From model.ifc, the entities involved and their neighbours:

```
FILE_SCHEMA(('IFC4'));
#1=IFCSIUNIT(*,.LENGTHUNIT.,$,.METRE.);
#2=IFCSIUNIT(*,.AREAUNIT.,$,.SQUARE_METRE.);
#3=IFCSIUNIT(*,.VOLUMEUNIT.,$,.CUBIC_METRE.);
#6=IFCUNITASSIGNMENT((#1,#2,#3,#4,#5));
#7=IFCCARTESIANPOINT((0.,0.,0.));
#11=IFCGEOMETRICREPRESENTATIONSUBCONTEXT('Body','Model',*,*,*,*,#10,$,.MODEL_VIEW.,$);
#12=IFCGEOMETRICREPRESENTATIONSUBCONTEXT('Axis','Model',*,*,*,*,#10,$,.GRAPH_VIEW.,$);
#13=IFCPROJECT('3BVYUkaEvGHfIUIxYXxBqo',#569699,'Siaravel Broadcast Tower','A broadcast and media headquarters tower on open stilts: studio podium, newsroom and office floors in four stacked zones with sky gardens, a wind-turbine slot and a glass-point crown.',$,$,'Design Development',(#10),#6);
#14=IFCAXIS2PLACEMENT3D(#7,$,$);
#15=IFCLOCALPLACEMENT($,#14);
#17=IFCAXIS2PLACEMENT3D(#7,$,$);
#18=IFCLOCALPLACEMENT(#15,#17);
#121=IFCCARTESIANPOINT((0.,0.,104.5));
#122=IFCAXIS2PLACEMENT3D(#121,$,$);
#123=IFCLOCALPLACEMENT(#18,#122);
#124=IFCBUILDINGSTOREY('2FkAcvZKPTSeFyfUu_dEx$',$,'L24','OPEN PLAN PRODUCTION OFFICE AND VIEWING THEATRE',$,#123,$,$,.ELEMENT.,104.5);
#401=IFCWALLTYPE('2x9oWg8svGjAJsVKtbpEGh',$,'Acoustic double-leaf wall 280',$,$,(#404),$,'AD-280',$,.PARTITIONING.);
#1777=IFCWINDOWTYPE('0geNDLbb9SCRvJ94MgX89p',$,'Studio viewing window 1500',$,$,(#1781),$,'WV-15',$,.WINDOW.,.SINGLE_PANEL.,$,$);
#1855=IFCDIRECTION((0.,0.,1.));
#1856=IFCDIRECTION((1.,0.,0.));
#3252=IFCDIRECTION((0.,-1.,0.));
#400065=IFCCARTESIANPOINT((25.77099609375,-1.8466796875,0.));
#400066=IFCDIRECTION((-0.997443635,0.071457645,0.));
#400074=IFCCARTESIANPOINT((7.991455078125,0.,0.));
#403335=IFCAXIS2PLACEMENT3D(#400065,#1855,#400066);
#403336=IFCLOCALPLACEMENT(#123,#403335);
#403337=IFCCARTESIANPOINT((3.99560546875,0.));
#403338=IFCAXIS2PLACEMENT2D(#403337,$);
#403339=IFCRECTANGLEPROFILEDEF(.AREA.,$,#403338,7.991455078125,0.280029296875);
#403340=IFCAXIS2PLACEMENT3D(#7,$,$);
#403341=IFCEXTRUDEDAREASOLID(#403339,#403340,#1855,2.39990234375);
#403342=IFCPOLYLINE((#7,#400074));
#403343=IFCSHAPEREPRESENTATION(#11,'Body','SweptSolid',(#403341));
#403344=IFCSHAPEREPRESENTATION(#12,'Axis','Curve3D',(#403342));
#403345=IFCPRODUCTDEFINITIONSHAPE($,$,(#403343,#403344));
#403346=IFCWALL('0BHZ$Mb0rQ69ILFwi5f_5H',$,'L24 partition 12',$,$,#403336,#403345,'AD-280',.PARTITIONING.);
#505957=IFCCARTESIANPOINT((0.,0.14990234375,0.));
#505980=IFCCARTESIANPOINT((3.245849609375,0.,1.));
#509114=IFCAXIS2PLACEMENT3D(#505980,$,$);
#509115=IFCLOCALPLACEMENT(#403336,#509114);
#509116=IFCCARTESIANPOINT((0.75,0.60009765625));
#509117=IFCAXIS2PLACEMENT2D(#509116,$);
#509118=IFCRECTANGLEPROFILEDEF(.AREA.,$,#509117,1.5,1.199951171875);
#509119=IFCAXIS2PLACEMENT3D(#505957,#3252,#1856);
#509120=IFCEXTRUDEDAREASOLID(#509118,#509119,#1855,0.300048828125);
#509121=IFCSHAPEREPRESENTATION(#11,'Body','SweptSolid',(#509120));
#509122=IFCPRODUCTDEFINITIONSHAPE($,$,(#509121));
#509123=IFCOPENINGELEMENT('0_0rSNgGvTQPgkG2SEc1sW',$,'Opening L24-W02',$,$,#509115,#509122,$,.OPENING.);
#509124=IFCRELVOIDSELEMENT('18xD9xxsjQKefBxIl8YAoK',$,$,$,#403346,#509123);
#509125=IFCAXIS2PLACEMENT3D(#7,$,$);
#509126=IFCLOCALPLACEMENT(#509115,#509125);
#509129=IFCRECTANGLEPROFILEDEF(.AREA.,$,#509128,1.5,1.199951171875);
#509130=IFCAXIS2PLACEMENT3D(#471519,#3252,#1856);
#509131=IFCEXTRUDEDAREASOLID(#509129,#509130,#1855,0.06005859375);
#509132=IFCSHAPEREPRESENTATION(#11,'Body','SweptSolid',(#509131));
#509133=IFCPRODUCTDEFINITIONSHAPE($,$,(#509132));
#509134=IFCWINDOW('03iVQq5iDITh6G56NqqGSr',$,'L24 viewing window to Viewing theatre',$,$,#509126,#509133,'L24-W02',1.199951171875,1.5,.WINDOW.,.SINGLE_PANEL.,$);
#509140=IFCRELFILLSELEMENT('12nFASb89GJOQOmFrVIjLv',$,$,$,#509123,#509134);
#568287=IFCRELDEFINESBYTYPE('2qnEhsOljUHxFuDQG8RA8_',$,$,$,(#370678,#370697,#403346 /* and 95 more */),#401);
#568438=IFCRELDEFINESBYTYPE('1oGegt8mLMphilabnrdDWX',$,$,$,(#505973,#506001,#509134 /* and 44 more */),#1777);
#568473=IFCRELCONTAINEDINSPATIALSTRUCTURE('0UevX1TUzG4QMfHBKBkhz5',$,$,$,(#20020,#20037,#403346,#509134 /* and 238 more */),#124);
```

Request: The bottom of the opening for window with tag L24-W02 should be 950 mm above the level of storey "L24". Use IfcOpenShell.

```python
import numpy as np
import ifcopenshell
import ifcopenshell.api.geometry
import ifcopenshell.geom
import ifcopenshell.util.element
import ifcopenshell.util.placement
import ifcopenshell.util.shape
import ifcopenshell.util.unit

model = ifcopenshell.open("model.ifc")
unit_scale = ifcopenshell.util.unit.calculate_unit_scale(model)

window = model.by_guid("03iVQq5iDITh6G56NqqGSr")
opening = window.FillsVoids[0].RelatingOpeningElement
storey = ifcopenshell.util.element.get_container(window, ifc_class="IfcBuildingStorey")
level = ifcopenshell.util.placement.get_local_placement(storey.ObjectPlacement)[2, 3]

# The opening's origin need not be at the sill, so measure its lowest point.
shape = ifcopenshell.geom.create_shape(ifcopenshell.geom.settings(), opening)
bottom = ifcopenshell.util.shape.get_shape_bottom_elevation(shape, shape.geometry) / unit_scale
dz = level + 0.95 / unit_scale - bottom

shift = np.array([0.0, 0.0, dz])
# The window is placed relative to its opening, so it follows when the opening moves.
matrix = ifcopenshell.util.placement.get_local_placement(opening.ObjectPlacement)
matrix[:3, 3] += shift
ifcopenshell.api.geometry.edit_object_placement(
    model, product=opening, matrix=matrix, is_si=False, should_transform_children=True
)

print(f"moved by {dz * unit_scale:+.3f} m")

model.write("model_edited.ifc")
```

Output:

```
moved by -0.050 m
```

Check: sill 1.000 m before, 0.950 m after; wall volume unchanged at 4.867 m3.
